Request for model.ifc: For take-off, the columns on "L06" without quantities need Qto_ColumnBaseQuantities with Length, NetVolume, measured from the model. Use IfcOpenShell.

First a look at what the model holds.

```python
import ifcopenshell
import ifcopenshell.util.element
import ifcopenshell.util.unit

model = ifcopenshell.open("model.ifc")
print(model.schema)
for unit_type in ("LENGTHUNIT", "AREAUNIT", "VOLUMEUNIT"):
    print(unit_type, ifcopenshell.util.unit.calculate_unit_scale(model, unit_type))
storey = next(s for s in model.by_type("IfcBuildingStorey") if s.Name == "L06")
columns = [e for e in ifcopenshell.util.element.get_decomposition(storey) if e.is_a("IfcColumn")]
for e in sorted(columns, key=lambda e: e.id()):
    print(e.id(), e.is_a(), e.Name, list(ifcopenshell.util.element.get_psets(e, qtos_only=True)), sep=" | ")
```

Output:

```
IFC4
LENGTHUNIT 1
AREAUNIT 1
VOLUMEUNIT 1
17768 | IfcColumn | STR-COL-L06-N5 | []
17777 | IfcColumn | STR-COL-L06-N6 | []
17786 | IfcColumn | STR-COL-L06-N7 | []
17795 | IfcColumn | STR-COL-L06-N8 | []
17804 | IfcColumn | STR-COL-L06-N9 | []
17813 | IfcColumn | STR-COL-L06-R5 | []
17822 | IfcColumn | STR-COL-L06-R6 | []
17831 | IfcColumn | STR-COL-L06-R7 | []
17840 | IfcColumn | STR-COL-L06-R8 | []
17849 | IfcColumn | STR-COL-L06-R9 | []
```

```python
import ifcopenshell
import ifcopenshell.api.pset
import ifcopenshell.geom
import ifcopenshell.util.element
import ifcopenshell.util.shape
import ifcopenshell.util.unit

model = ifcopenshell.open("model.ifc")
unit_scale = ifcopenshell.util.unit.calculate_unit_scale(model)
volume_scale = ifcopenshell.util.unit.calculate_unit_scale(model, "VOLUMEUNIT")
settings = ifcopenshell.geom.settings()

storey = next(s for s in model.by_type("IfcBuildingStorey") if s.Name == "L06")
columns = [e for e in ifcopenshell.util.element.get_decomposition(storey) if e.is_a("IfcColumn")]

for e in sorted(columns, key=lambda e: e.id()):
    if ifcopenshell.util.element.get_psets(e, qtos_only=True, should_inherit=False):
        continue
    # Geometry comes back in metres, in the element's own axes.
    shape = ifcopenshell.geom.create_shape(settings, e)
    values = {
        "Length": ifcopenshell.util.shape.get_z(shape.geometry) / unit_scale,
        "NetVolume": ifcopenshell.util.shape.get_volume(shape.geometry) / volume_scale,
    }
    qto = ifcopenshell.api.pset.add_qto(model, product=e, name="Qto_ColumnBaseQuantities")
    ifcopenshell.api.pset.edit_qto(model, qto=qto, properties=values)
    print(e.id(), {k: round(v, 3) for k, v in values.items()})

model.write("model_rev.ifc")
```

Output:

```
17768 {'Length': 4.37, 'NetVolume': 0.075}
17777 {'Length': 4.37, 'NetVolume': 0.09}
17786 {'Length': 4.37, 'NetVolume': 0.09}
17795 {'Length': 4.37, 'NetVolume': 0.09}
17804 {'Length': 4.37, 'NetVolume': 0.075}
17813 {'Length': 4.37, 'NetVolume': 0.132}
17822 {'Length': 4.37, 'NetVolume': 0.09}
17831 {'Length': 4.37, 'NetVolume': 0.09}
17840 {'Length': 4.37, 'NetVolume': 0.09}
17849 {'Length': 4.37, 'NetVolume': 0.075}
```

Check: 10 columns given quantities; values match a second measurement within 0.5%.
